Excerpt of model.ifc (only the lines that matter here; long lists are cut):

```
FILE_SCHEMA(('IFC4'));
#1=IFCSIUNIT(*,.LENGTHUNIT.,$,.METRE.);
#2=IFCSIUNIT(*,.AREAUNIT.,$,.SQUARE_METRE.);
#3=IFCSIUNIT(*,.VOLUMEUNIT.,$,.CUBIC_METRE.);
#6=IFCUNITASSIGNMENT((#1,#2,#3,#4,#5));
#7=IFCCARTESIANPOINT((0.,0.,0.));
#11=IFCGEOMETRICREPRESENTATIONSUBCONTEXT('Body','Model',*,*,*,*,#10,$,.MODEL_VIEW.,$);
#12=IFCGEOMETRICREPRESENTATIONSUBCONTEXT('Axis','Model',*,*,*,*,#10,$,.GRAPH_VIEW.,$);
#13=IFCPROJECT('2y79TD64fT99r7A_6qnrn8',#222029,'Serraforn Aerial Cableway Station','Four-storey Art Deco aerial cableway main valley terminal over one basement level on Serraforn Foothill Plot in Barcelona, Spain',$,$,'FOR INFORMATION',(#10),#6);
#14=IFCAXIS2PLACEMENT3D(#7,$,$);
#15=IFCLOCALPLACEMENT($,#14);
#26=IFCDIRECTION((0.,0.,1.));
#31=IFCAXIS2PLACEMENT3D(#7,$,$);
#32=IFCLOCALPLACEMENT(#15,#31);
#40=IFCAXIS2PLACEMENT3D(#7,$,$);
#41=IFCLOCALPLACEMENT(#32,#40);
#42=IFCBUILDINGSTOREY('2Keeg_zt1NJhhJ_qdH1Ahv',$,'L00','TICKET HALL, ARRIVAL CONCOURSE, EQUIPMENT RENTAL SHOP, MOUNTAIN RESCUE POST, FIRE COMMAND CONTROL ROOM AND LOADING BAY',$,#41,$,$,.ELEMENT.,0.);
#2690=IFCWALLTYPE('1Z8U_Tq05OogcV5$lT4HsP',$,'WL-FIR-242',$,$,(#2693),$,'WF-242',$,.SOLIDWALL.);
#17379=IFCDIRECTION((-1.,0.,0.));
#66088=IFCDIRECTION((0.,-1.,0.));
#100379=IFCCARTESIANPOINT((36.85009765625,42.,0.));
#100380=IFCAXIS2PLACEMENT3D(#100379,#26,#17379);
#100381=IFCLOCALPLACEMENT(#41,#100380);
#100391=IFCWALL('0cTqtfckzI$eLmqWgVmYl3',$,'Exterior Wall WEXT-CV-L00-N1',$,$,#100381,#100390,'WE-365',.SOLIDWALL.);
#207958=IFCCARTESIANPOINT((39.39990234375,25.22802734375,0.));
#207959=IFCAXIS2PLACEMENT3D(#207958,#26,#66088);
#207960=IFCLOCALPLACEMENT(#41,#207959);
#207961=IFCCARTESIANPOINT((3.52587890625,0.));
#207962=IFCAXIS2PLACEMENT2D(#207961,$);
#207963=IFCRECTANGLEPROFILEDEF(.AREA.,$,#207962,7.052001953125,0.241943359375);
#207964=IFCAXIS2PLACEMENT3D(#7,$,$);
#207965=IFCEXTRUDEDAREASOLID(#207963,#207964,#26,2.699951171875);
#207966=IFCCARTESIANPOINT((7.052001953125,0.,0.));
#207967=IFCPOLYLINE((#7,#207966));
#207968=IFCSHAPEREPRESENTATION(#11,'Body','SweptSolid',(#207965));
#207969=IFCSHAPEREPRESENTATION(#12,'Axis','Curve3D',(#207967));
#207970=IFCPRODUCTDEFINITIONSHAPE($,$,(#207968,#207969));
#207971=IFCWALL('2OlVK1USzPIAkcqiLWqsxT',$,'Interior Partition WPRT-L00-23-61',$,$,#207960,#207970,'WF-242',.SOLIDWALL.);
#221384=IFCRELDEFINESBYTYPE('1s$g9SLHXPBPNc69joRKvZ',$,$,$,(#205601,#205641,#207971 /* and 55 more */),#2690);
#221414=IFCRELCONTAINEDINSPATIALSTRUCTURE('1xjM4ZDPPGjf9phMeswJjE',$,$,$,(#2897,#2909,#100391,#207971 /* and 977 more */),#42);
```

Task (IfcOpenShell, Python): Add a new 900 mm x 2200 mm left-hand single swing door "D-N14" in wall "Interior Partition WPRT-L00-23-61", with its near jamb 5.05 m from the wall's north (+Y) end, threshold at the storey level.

```python
import numpy as np
import ifcopenshell
import ifcopenshell.api.feature
import ifcopenshell.api.geometry
import ifcopenshell.api.root
import ifcopenshell.api.spatial
import ifcopenshell.geom
import ifcopenshell.util.element
import ifcopenshell.util.placement
import ifcopenshell.util.representation
import ifcopenshell.util.shape
import ifcopenshell.util.unit

model = ifcopenshell.open("model.ifc")
unit_scale = ifcopenshell.util.unit.calculate_unit_scale(model)
settings = ifcopenshell.geom.settings()


def volume(element):
    """Net volume in cubic metres, openings subtracted."""
    shape = ifcopenshell.geom.create_shape(settings, element)
    return ifcopenshell.util.shape.get_volume(shape.geometry)


wall = model.by_guid("2OlVK1USzPIAkcqiLWqsxT")
storey = ifcopenshell.util.element.get_container(wall, ifc_class="IfcBuildingStorey")
context = ifcopenshell.util.representation.get_context(model, "Model", "Body", "MODEL_VIEW")
before = volume(wall)

width, height, from_end, sill = 0.9, 2.2, 5.05, 0.0  # metres

# The wall runs along its own X axis, and the end named is its -X end.
wall_shape = ifcopenshell.geom.create_shape(settings, wall)
x, y, z = ifcopenshell.util.shape.get_vertices(wall_shape.geometry).T
start = x.min() + from_end
face, thickness = float(y.min()), float(y.max() - y.min())
wall_matrix = ifcopenshell.util.placement.get_local_placement(wall.ObjectPlacement)
level = ifcopenshell.util.placement.get_local_placement(storey.ObjectPlacement)[2, 3]


def in_wall(x, y):
    """Placement at x, y metres in the wall's axes, at sill height."""
    matrix = wall_matrix.copy()
    matrix[:, 3] = wall_matrix @ np.array([x / unit_scale, y / unit_scale, 0.0, 1.0])
    matrix[2, 3] = level + sill / unit_scale
    return matrix


# Opening: a box that overshoots both wall faces by 50 mm.
opening = ifcopenshell.api.root.create_entity(model, ifc_class="IfcOpeningElement", predefined_type="OPENING")
box = ifcopenshell.api.geometry.add_wall_representation(
    model, context=context, length=width, height=height, thickness=thickness + 0.1
)
ifcopenshell.api.geometry.assign_representation(model, product=opening, representation=box)
ifcopenshell.api.geometry.edit_object_placement(model, product=opening, matrix=in_wall(start, face - 0.05), is_si=False)
ifcopenshell.api.feature.add_feature(model, feature=opening, element=wall)

door = ifcopenshell.api.root.create_entity(model, ifc_class="IfcDoor", name="D-N14", predefined_type="DOOR")
door.OverallWidth, door.OverallHeight = width / unit_scale, height / unit_scale
door.OperationType = "SINGLE_SWING_LEFT"
body = ifcopenshell.api.geometry.add_door_representation(
    model,
    context=context,
    overall_width=door.OverallWidth,
    overall_height=door.OverallHeight,
    operation_type="SINGLE_SWING_LEFT",
    lining_properties={"LiningDepth": thickness / unit_scale, "ThresholdDepth": thickness / unit_scale},
)
ifcopenshell.api.geometry.assign_representation(model, product=door, representation=body)
ifcopenshell.api.spatial.assign_container(model, products=[door], relating_structure=storey)
ifcopenshell.api.feature.add_filling(model, opening=opening, element=door)

# The lining spans the wall, so the door starts at the wall face.
ifcopenshell.api.geometry.edit_object_placement(model, product=door, matrix=in_wall(start, face), is_si=False)

after = volume(wall)

print(f"wall volume {before:.3f} -> {after:.3f} m3")

model.write("model_v2.ifc")
```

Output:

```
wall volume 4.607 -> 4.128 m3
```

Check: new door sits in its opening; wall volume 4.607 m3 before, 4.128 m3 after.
